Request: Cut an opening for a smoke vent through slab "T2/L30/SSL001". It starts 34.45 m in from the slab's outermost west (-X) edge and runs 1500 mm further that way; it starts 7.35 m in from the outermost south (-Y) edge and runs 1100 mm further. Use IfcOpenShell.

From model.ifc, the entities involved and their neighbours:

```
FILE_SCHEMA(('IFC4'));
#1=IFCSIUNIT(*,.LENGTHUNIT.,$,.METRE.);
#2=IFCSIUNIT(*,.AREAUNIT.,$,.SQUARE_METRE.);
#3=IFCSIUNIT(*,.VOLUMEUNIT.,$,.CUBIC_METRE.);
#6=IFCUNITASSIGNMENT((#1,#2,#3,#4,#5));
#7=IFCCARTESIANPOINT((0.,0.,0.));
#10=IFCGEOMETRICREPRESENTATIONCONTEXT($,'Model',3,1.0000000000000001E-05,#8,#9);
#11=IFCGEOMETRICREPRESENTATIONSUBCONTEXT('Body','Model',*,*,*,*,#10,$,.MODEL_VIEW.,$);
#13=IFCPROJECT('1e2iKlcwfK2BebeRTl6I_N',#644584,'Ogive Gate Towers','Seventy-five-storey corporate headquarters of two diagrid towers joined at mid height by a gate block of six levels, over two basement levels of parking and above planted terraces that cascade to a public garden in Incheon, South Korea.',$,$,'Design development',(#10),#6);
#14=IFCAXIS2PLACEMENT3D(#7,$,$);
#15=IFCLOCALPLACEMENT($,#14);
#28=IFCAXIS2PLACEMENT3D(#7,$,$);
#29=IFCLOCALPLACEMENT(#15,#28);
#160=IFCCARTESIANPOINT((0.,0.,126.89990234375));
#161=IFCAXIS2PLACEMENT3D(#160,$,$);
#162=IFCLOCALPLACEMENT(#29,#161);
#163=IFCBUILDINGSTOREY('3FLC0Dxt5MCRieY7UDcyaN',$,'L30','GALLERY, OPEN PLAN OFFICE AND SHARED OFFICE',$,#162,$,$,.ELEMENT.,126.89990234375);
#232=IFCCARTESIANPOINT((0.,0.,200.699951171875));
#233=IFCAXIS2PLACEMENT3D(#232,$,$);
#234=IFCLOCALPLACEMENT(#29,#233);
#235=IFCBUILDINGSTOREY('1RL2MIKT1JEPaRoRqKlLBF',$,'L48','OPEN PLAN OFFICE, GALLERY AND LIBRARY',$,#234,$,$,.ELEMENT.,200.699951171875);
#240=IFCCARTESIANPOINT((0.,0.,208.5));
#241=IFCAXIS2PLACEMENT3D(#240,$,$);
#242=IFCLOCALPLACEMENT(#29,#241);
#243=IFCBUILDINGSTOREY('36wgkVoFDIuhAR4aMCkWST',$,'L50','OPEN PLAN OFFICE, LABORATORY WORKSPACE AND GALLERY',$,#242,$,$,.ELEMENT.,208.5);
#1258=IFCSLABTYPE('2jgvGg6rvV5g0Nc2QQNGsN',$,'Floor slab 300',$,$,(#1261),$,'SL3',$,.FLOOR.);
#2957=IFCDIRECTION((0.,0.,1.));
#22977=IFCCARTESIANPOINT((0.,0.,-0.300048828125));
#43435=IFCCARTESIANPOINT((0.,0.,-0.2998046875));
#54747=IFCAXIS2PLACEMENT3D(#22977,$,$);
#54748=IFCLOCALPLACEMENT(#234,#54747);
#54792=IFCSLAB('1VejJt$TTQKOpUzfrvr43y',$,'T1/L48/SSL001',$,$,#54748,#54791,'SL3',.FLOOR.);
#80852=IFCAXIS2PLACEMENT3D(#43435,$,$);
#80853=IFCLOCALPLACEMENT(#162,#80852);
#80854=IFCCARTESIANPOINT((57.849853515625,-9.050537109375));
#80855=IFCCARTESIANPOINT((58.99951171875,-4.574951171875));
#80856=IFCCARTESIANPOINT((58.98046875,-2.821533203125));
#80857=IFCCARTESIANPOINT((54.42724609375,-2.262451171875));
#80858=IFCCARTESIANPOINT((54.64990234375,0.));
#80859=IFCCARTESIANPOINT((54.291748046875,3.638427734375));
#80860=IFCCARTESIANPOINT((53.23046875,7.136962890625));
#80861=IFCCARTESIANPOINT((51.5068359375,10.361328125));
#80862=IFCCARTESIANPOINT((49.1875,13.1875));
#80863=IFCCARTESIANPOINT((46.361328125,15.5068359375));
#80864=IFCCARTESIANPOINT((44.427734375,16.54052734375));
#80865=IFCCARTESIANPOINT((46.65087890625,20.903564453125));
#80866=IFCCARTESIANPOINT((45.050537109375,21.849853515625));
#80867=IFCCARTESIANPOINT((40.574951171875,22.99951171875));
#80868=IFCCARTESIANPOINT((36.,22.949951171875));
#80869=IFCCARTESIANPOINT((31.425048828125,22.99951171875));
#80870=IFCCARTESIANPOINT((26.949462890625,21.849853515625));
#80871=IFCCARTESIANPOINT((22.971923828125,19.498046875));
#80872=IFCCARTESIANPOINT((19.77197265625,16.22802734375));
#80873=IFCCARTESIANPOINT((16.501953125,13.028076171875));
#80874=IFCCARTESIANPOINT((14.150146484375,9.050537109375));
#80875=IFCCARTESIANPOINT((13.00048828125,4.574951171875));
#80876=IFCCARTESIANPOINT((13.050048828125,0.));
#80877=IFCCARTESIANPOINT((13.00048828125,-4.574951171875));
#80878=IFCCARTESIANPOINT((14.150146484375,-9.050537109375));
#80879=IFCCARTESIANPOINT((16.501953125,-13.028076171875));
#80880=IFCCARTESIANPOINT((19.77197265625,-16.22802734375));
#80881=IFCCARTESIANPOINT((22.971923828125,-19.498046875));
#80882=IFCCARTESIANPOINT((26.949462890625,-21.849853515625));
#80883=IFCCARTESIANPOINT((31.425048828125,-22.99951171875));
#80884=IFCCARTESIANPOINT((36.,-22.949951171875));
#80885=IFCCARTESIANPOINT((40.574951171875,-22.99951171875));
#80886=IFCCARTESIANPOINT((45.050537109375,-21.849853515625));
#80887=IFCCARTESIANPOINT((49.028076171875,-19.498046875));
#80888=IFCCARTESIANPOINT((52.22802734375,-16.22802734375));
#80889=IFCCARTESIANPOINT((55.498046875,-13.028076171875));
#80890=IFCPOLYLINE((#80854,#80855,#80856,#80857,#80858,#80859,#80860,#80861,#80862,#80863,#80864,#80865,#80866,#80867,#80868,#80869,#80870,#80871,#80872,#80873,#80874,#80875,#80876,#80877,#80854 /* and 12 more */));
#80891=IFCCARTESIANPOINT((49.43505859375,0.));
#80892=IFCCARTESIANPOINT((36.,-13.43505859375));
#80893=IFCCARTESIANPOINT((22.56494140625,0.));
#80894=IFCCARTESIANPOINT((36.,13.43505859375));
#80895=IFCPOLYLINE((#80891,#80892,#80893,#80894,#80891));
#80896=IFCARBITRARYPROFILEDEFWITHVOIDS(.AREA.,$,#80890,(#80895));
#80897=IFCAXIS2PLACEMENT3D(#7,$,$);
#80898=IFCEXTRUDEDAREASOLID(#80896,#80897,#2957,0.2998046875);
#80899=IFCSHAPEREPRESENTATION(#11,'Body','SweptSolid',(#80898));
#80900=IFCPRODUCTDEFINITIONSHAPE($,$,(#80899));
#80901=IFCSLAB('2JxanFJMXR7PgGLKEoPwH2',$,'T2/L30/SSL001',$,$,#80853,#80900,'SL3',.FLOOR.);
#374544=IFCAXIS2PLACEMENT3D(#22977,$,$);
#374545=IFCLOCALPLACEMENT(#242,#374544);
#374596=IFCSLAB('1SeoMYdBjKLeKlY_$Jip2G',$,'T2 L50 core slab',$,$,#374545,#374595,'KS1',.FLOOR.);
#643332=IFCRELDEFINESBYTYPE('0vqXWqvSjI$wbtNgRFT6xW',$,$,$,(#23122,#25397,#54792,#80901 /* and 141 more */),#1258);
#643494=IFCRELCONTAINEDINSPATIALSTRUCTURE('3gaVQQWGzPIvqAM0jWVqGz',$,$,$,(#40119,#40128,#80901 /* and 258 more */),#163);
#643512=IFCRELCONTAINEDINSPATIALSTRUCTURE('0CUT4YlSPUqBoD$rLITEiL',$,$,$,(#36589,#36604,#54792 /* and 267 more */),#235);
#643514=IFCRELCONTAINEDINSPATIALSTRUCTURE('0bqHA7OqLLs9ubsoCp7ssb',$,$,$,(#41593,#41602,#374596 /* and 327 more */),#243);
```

```python
import numpy as np
import ifcopenshell
import ifcopenshell.api.feature
import ifcopenshell.api.geometry
import ifcopenshell.api.root
import ifcopenshell.geom
import ifcopenshell.util.placement
import ifcopenshell.util.representation
import ifcopenshell.util.shape
import ifcopenshell.util.unit

model = ifcopenshell.open("model.ifc")
unit_scale = ifcopenshell.util.unit.calculate_unit_scale(model)
settings = ifcopenshell.geom.settings()


def volume(element):
    """Net volume in cubic metres, openings subtracted."""
    shape = ifcopenshell.geom.create_shape(settings, element)
    return ifcopenshell.util.shape.get_volume(shape.geometry)


slab = model.by_id(80901)
before = volume(slab)

# Extent in the slab's own axes, in metres. The edges named are its -X and -Y sides.
slab_shape = ifcopenshell.geom.create_shape(settings, slab)
vertices = ifcopenshell.util.shape.get_vertices(slab_shape.geometry)
x_min, y_min, bottom = vertices.min(axis=0)
top = vertices[:, 2].max()

opening = ifcopenshell.api.root.create_entity(model, ifc_class="IfcOpeningElement", name="Smoke vent opening", predefined_type="OPENING")
context = ifcopenshell.util.representation.get_context(model, "Model", "Body", "MODEL_VIEW")
width, depth = 1.5, 1.1
outline = [(0.0, 0.0), (width, 0.0), (width, depth), (0.0, depth), (0.0, 0.0)]
# Overshoot both faces by 50 mm so the cut is clean.
shape = ifcopenshell.api.geometry.add_slab_representation(
    model, context=context, depth=top - bottom + 0.1, polyline=outline
)
ifcopenshell.api.geometry.assign_representation(model, product=opening, representation=shape)

matrix = ifcopenshell.util.placement.get_local_placement(slab.ObjectPlacement)
matrix[:, 3] = matrix @ np.append(np.array([x_min + 34.45, y_min + 7.35, bottom - 0.05]) / unit_scale, 1.0)
ifcopenshell.api.geometry.edit_object_placement(model, product=opening, matrix=matrix, is_si=False)
ifcopenshell.api.feature.add_feature(model, feature=opening, element=slab)

after = volume(slab)

print(f"slab volume {before:.3f} -> {after:.3f} m3")

model.write("model_v2.ifc")
```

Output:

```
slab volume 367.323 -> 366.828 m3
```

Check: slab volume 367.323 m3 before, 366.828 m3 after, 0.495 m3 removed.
